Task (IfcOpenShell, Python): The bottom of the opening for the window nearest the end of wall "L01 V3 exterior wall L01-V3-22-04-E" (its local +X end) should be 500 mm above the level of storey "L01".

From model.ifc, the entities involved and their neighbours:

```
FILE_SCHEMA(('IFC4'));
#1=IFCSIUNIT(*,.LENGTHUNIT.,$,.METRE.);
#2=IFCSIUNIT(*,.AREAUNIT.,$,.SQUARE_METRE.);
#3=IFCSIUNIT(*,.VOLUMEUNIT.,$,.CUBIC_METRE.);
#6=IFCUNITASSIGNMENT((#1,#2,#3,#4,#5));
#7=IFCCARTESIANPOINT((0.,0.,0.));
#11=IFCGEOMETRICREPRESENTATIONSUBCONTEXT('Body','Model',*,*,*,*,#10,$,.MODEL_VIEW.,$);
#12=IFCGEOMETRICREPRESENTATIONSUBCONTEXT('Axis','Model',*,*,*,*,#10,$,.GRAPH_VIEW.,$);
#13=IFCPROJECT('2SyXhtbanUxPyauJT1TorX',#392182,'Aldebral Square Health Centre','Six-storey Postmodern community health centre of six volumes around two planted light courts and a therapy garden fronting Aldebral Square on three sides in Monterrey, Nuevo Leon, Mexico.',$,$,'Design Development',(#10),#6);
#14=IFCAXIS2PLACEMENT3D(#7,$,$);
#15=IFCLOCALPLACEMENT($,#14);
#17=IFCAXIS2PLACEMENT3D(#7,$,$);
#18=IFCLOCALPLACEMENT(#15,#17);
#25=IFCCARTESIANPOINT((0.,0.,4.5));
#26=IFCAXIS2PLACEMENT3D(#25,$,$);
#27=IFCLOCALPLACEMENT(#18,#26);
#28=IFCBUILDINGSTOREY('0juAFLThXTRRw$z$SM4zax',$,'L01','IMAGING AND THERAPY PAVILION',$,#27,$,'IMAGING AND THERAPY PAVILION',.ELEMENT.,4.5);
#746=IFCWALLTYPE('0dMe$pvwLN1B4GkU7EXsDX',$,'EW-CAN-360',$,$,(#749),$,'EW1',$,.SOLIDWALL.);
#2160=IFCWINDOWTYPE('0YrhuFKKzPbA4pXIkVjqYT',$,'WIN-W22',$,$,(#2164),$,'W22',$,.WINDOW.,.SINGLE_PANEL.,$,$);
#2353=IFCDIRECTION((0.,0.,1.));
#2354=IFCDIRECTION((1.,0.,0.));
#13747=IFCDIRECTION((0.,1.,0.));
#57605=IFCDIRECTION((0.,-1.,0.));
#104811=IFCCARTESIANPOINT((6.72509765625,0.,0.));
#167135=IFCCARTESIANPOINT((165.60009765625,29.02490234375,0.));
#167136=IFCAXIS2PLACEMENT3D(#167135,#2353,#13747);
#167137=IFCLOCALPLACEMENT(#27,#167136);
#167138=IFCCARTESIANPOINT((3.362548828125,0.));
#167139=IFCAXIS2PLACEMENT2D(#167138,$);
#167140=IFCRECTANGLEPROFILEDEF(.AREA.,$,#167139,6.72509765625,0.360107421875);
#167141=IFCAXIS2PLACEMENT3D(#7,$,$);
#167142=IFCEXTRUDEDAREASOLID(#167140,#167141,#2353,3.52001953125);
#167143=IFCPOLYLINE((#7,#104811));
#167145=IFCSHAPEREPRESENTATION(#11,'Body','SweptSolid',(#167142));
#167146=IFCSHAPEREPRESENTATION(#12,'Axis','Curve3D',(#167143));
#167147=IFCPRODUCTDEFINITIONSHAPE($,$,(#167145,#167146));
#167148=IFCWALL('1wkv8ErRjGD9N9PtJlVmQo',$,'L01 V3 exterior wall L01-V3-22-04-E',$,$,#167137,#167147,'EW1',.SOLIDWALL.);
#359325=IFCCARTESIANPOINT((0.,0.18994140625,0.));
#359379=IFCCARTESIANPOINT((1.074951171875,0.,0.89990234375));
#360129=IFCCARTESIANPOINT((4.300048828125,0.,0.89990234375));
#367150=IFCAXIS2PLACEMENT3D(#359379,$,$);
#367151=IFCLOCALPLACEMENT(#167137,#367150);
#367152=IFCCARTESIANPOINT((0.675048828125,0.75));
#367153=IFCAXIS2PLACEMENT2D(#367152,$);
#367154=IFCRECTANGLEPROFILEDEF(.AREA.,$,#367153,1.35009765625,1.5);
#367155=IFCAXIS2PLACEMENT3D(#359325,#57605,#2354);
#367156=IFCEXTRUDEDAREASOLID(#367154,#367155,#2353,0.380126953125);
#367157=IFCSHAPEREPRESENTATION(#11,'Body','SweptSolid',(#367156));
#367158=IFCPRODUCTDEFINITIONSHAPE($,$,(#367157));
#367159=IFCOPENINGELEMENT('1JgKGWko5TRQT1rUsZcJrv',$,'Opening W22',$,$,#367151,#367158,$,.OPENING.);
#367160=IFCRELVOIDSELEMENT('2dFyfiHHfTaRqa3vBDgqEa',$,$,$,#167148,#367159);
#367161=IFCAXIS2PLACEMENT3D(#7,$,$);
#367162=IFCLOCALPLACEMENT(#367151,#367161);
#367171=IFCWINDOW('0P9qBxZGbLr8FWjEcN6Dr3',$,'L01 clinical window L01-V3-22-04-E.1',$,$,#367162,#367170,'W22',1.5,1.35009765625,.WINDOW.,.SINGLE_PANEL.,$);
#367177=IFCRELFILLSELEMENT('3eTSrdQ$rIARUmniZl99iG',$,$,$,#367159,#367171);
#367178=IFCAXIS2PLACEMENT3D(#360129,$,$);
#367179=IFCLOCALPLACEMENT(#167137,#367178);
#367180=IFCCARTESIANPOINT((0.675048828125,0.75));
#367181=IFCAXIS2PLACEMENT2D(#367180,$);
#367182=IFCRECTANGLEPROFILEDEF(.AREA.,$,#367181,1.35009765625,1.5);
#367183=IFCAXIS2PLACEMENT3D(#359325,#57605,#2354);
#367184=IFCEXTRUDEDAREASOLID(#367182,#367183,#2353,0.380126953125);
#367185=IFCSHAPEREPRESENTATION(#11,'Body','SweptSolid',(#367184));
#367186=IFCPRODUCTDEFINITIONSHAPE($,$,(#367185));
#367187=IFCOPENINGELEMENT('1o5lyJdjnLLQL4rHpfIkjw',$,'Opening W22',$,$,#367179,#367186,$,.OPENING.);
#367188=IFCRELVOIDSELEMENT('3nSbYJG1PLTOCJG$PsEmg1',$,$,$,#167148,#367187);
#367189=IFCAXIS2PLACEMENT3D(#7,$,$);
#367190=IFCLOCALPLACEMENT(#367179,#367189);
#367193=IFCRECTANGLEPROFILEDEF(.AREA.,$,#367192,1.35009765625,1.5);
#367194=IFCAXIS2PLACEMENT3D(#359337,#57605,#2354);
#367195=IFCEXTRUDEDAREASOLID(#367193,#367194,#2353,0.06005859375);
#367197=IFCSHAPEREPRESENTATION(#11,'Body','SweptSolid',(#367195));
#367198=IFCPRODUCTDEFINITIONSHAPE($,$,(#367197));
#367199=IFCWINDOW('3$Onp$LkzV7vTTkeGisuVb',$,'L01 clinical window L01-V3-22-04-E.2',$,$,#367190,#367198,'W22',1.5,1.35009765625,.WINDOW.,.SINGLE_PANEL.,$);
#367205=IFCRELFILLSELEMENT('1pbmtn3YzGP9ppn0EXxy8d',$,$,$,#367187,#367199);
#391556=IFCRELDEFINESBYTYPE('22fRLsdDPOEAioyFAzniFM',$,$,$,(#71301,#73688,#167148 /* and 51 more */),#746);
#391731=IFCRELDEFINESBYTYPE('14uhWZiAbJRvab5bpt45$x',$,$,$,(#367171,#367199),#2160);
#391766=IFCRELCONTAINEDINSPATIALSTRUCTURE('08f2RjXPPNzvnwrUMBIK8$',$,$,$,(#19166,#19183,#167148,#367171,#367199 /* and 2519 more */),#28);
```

```python
import numpy as np
import ifcopenshell
import ifcopenshell.api.geometry
import ifcopenshell.geom
import ifcopenshell.util.element
import ifcopenshell.util.placement
import ifcopenshell.util.shape
import ifcopenshell.util.unit

model = ifcopenshell.open("model.ifc")
unit_scale = ifcopenshell.util.unit.calculate_unit_scale(model)

window = model.by_id(367199)
opening = window.FillsVoids[0].RelatingOpeningElement
storey = ifcopenshell.util.element.get_container(window, ifc_class="IfcBuildingStorey")
level = ifcopenshell.util.placement.get_local_placement(storey.ObjectPlacement)[2, 3]

# The opening's origin need not be at the sill, so measure its lowest point.
shape = ifcopenshell.geom.create_shape(ifcopenshell.geom.settings(), opening)
bottom = ifcopenshell.util.shape.get_shape_bottom_elevation(shape, shape.geometry) / unit_scale
dz = level + 0.5 - bottom

shift = np.array([0.0, 0.0, dz])
# The window is placed relative to its opening, so it follows when the opening moves.
matrix = ifcopenshell.util.placement.get_local_placement(opening.ObjectPlacement)
matrix[:3, 3] += shift
ifcopenshell.api.geometry.edit_object_placement(
    model, product=opening, matrix=matrix, is_si=False, should_transform_children=True
)

print(f"moved by {dz * unit_scale:+.3f} m")

model.write("model_updated.ifc")
```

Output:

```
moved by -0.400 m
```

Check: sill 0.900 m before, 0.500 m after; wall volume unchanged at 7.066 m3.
